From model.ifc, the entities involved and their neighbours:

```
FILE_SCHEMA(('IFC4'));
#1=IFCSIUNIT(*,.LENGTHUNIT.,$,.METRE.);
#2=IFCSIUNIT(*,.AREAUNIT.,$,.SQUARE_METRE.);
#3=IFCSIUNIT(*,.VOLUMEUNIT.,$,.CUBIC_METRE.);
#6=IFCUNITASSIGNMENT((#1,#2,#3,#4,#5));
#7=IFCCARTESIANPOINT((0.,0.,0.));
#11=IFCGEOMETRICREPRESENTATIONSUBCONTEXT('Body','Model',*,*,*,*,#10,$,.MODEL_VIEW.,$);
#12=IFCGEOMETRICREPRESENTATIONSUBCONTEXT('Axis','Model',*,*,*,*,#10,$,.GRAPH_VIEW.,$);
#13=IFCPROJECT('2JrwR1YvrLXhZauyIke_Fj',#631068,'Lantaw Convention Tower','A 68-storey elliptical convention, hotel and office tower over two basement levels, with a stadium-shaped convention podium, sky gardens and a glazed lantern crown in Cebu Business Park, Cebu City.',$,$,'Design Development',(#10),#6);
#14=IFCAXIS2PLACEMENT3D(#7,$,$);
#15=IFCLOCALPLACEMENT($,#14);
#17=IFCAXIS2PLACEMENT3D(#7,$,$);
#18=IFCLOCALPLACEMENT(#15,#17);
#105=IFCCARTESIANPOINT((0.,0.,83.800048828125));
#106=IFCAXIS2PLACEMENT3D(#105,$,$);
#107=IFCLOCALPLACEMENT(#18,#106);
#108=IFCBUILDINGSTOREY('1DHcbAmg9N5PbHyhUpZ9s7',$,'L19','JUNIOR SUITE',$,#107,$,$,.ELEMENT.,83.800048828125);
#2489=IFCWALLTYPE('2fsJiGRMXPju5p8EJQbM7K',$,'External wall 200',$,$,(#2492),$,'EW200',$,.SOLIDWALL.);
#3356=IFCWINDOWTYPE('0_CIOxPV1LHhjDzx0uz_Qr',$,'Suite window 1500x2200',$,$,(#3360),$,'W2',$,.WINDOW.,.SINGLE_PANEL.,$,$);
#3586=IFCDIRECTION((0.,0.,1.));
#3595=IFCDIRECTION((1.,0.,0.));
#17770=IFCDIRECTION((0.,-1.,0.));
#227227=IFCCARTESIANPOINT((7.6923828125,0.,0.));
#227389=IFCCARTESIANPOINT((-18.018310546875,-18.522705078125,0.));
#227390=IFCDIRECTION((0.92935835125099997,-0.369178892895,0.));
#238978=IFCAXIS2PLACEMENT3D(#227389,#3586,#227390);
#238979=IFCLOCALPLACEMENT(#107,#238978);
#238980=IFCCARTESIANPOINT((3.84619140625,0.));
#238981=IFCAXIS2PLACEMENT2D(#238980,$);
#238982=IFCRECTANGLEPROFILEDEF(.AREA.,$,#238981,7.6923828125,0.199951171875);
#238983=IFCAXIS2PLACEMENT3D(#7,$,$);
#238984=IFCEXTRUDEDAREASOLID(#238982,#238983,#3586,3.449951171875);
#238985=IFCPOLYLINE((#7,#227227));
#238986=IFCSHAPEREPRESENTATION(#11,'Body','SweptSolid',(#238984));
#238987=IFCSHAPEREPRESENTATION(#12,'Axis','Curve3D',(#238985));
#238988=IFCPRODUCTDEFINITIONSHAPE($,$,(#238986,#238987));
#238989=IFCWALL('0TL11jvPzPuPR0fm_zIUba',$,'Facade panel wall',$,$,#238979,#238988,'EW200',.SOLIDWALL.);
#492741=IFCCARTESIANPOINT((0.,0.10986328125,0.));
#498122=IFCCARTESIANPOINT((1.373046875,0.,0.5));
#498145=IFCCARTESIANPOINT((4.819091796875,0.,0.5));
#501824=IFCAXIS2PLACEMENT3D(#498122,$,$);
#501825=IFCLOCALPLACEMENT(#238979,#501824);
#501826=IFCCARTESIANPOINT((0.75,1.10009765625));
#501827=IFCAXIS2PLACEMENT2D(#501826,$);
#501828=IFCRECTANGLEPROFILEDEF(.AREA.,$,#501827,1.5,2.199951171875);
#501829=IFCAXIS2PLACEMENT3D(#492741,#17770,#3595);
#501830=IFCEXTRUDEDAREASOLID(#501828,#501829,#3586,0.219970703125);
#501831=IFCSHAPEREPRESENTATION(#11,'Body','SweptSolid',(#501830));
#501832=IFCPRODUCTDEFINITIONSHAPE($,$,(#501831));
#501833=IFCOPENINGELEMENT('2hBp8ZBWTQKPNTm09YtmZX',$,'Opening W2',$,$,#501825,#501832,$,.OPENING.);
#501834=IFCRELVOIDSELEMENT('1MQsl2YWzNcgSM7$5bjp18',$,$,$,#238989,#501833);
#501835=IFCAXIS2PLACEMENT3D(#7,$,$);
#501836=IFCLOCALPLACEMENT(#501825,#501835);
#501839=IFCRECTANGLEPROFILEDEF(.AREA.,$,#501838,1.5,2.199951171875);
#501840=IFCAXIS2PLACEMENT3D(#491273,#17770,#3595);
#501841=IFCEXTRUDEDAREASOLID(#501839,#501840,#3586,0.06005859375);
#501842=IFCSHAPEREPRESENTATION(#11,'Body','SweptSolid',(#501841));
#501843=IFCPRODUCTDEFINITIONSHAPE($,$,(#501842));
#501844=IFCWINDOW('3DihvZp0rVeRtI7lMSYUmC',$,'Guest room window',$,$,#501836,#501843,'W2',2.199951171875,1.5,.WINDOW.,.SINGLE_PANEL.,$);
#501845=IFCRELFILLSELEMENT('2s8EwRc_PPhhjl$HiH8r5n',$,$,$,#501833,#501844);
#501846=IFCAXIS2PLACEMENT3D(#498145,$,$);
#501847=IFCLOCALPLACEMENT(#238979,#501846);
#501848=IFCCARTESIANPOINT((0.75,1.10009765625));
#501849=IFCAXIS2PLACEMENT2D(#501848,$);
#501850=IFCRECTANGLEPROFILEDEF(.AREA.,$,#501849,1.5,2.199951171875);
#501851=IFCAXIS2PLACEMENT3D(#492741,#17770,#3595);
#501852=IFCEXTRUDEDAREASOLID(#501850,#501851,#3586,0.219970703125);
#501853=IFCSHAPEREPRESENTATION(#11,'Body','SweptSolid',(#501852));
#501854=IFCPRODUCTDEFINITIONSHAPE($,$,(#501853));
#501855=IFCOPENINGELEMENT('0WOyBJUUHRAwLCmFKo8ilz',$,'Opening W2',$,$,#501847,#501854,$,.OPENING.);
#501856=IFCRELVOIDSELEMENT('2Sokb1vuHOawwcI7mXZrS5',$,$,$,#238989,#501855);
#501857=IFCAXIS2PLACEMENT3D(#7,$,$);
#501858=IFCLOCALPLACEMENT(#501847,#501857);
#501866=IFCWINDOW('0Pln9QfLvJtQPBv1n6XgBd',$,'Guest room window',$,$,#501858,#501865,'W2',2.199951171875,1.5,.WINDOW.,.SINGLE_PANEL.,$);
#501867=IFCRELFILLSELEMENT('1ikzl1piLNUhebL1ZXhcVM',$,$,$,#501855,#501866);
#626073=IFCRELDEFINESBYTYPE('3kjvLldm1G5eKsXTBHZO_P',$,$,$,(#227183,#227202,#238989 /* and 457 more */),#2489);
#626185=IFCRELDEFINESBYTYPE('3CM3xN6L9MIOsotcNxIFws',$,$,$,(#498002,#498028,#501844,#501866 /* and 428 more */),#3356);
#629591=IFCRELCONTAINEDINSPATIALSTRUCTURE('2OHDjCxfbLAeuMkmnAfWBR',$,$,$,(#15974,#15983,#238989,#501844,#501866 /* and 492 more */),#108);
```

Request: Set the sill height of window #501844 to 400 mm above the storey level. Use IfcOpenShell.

```python
import numpy as np
import ifcopenshell
import ifcopenshell.api.geometry
import ifcopenshell.geom
import ifcopenshell.util.element
import ifcopenshell.util.placement
import ifcopenshell.util.shape
import ifcopenshell.util.unit

model = ifcopenshell.open("model.ifc")
unit_scale = ifcopenshell.util.unit.calculate_unit_scale(model)

window = model.by_guid("3DihvZp0rVeRtI7lMSYUmC")
opening = window.FillsVoids[0].RelatingOpeningElement
storey = ifcopenshell.util.element.get_container(window, ifc_class="IfcBuildingStorey")
level = ifcopenshell.util.placement.get_local_placement(storey.ObjectPlacement)[2, 3]

# The opening's origin need not be at the sill, so measure its lowest point.
shape = ifcopenshell.geom.create_shape(ifcopenshell.geom.settings(), opening)
bottom = ifcopenshell.util.shape.get_shape_bottom_elevation(shape, shape.geometry) / unit_scale
dz = level + 0.4 / unit_scale - bottom

shift = np.array([0.0, 0.0, dz])
# The window is placed relative to its opening, so it follows when the opening moves.
matrix = ifcopenshell.util.placement.get_local_placement(opening.ObjectPlacement)
matrix[:3, 3] += shift
ifcopenshell.api.geometry.edit_object_placement(
    model, product=opening, matrix=matrix, is_si=False, should_transform_children=True
)

print(f"moved by {dz * unit_scale:+.3f} m")

model.write("model_updated.ifc")
```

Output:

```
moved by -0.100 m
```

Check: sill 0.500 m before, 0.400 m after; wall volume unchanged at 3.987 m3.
